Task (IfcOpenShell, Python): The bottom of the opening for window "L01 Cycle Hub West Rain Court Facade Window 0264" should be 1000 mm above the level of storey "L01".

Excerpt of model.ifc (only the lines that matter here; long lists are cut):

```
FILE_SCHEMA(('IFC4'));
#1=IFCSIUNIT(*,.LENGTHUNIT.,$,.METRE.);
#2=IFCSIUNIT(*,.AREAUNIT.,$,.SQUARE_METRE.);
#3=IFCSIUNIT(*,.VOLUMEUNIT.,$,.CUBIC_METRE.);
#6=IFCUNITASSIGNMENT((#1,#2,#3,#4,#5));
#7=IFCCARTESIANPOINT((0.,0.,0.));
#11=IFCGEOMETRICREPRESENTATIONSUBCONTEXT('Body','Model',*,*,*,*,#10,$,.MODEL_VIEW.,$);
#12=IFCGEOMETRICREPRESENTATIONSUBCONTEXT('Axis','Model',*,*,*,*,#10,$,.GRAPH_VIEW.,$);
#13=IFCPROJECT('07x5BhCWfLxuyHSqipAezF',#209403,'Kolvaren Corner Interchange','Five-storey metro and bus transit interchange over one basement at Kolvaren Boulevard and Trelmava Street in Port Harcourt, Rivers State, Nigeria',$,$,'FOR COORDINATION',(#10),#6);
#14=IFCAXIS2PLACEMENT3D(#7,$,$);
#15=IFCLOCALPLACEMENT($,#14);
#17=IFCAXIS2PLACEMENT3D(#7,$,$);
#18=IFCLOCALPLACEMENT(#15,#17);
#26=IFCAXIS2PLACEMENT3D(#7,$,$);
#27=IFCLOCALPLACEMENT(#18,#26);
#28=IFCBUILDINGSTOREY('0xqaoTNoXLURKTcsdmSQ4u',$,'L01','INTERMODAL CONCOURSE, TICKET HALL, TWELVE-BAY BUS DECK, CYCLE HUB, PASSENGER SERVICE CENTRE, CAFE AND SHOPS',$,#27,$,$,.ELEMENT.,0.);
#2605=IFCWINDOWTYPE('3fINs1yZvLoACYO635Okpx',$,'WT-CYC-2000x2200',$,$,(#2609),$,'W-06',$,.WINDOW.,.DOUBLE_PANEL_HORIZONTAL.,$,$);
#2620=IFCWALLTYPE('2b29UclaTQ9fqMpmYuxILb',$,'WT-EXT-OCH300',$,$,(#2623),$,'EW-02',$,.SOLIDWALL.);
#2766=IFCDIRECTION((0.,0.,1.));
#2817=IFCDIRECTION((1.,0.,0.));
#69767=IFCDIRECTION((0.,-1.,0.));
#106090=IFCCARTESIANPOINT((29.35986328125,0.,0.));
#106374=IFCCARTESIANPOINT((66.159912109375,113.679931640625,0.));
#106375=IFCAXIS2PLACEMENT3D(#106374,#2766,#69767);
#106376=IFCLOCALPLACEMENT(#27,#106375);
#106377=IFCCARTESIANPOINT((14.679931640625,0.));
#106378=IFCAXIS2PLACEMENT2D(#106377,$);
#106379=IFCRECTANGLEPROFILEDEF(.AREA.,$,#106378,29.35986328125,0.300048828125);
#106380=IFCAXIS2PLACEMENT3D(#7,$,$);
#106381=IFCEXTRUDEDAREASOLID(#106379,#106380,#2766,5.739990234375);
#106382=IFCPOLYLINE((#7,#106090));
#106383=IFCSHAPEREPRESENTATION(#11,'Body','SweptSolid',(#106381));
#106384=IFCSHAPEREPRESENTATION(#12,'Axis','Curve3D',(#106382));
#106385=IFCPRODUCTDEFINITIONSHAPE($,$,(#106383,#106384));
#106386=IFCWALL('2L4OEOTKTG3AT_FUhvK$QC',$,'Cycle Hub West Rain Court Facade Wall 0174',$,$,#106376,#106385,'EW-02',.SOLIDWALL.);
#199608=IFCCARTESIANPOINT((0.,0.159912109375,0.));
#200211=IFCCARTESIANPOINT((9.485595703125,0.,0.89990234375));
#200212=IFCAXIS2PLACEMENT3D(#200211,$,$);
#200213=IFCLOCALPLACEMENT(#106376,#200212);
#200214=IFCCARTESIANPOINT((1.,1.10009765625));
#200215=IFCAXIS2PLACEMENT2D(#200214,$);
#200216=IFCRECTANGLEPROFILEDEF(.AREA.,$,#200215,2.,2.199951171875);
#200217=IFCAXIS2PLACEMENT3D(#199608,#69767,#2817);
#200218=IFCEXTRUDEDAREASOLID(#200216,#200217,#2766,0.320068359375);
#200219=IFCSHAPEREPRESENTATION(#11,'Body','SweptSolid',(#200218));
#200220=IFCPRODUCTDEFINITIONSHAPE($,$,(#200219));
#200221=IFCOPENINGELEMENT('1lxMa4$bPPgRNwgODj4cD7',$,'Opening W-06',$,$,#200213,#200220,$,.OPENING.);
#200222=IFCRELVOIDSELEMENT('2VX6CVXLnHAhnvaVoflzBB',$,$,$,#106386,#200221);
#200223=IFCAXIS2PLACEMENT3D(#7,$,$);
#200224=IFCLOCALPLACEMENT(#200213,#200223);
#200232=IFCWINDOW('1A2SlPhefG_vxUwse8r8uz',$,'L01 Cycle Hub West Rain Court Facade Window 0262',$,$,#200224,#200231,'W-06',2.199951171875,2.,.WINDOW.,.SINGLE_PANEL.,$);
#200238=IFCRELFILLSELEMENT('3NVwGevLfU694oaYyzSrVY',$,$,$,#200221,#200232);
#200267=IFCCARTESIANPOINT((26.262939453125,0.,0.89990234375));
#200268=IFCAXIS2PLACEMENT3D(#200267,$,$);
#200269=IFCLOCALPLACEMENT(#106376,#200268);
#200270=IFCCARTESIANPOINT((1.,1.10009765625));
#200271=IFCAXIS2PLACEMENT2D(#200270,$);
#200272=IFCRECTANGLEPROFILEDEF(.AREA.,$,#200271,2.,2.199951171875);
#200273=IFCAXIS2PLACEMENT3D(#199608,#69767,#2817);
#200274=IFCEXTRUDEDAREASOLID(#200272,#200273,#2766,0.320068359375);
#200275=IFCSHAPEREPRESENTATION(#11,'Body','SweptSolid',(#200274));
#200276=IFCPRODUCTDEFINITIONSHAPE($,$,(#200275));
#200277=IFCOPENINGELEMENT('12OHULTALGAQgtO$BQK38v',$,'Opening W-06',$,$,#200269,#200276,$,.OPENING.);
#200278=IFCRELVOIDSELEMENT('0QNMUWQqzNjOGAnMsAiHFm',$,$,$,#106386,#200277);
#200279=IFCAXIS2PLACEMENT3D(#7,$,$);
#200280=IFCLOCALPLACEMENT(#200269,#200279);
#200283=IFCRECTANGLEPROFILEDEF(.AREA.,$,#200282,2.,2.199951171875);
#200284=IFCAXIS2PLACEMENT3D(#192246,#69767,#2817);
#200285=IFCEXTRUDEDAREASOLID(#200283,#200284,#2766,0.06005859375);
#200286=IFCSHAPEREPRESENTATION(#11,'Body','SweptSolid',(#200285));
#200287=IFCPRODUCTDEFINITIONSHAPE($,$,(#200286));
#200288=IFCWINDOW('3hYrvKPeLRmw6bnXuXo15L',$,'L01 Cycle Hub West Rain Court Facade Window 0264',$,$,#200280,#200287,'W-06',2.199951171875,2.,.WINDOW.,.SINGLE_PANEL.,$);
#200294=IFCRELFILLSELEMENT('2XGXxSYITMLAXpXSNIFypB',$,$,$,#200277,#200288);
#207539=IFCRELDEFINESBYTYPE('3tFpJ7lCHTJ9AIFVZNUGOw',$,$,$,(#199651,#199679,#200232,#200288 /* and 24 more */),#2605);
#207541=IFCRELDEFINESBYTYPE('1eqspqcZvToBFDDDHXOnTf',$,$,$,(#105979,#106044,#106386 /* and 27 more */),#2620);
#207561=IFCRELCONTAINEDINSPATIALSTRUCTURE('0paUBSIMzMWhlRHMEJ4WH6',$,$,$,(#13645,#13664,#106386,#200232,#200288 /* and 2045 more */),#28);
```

```python
import numpy as np
import ifcopenshell
import ifcopenshell.api.geometry
import ifcopenshell.geom
import ifcopenshell.util.element
import ifcopenshell.util.placement
import ifcopenshell.util.shape
import ifcopenshell.util.unit

model = ifcopenshell.open("model.ifc")
unit_scale = ifcopenshell.util.unit.calculate_unit_scale(model)

window = model.by_guid("3hYrvKPeLRmw6bnXuXo15L")
opening = window.FillsVoids[0].RelatingOpeningElement
storey = ifcopenshell.util.element.get_container(window, ifc_class="IfcBuildingStorey")
level = ifcopenshell.util.placement.get_local_placement(storey.ObjectPlacement)[2, 3]

# The opening's origin need not be at the sill, so measure its lowest point.
shape = ifcopenshell.geom.create_shape(ifcopenshell.geom.settings(), opening)
bottom = ifcopenshell.util.shape.get_shape_bottom_elevation(shape, shape.geometry) / unit_scale
dz = level + 1.0 - bottom

shift = np.array([0.0, 0.0, dz])
# The window is placed relative to its opening, so it follows when the opening moves.
matrix = ifcopenshell.util.placement.get_local_placement(opening.ObjectPlacement)
matrix[:3, 3] += shift
ifcopenshell.api.geometry.edit_object_placement(
    model, product=opening, matrix=matrix, is_si=False, should_transform_children=True
)

print(f"moved by {dz * unit_scale:+.3f} m")

model.write("model_edited.ifc")
```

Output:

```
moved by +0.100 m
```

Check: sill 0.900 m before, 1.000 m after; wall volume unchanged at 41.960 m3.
